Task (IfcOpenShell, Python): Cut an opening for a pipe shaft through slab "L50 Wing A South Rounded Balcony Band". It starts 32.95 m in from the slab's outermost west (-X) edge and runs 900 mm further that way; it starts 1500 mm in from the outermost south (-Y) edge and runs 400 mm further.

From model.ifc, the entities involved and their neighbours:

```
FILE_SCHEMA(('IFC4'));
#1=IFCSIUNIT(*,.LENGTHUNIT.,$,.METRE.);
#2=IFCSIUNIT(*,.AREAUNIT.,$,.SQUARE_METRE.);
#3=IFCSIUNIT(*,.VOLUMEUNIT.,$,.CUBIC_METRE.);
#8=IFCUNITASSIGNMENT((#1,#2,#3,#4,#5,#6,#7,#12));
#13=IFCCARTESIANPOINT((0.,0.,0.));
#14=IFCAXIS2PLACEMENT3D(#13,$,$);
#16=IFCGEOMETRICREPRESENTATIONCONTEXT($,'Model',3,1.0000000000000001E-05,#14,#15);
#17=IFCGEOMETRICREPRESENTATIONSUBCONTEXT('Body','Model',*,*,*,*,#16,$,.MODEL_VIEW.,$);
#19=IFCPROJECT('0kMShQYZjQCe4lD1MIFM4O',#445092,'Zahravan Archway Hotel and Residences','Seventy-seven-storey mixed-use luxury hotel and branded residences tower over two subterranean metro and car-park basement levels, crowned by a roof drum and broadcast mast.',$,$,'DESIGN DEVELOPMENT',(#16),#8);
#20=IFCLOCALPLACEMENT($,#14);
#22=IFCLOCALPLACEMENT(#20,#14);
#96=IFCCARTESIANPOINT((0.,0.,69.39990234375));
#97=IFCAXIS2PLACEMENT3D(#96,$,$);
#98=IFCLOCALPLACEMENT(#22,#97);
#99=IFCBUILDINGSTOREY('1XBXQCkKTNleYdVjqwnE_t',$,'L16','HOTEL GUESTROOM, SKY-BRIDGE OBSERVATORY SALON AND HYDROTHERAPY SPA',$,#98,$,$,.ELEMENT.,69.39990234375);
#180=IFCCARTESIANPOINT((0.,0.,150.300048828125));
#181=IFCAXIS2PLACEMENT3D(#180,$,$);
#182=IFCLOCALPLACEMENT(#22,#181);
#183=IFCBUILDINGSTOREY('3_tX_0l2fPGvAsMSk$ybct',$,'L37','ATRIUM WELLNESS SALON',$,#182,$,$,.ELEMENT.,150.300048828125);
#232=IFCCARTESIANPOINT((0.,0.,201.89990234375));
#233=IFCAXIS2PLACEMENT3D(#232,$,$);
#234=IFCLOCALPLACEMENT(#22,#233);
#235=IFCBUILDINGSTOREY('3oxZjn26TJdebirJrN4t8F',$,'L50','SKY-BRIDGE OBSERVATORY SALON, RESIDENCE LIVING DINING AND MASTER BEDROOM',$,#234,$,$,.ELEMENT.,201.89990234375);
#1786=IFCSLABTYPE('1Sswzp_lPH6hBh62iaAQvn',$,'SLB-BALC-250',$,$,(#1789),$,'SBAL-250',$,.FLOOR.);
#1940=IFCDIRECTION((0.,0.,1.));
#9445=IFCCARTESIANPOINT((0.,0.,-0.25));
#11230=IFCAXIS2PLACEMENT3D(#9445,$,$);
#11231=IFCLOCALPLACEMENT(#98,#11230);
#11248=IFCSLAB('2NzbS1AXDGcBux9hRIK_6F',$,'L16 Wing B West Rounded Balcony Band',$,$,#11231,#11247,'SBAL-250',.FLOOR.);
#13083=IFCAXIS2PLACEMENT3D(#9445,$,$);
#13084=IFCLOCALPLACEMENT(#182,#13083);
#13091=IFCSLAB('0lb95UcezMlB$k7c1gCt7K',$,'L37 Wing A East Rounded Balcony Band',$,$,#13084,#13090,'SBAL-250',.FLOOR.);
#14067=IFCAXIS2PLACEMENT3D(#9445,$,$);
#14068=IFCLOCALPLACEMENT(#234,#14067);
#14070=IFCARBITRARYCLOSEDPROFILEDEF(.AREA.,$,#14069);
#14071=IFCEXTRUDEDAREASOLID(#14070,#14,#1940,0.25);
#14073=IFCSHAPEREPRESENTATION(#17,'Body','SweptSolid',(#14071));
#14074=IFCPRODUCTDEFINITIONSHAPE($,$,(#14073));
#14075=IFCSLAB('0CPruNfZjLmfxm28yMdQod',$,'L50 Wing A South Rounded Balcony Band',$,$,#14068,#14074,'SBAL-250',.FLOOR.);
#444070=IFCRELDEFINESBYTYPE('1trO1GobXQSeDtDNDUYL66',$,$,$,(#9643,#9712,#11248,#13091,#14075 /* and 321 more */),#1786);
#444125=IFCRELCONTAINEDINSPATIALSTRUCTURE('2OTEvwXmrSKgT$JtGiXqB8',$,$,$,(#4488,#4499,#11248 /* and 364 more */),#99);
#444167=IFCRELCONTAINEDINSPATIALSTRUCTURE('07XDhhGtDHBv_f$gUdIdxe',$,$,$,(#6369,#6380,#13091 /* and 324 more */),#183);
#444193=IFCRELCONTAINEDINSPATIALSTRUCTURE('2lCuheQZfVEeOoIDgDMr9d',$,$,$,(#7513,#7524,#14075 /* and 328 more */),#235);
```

```python
import numpy as np
import ifcopenshell
import ifcopenshell.api.feature
import ifcopenshell.api.geometry
import ifcopenshell.api.root
import ifcopenshell.geom
import ifcopenshell.util.placement
import ifcopenshell.util.representation
import ifcopenshell.util.shape
import ifcopenshell.util.unit

model = ifcopenshell.open("model.ifc")
unit_scale = ifcopenshell.util.unit.calculate_unit_scale(model)
settings = ifcopenshell.geom.settings()


def volume(element):
    """Net volume in cubic metres, openings subtracted."""
    shape = ifcopenshell.geom.create_shape(settings, element)
    return ifcopenshell.util.shape.get_volume(shape.geometry)


slab = model.by_guid("0CPruNfZjLmfxm28yMdQod")
before = volume(slab)

# Extent in the slab's own axes, in metres. The edges named are its -X and -Y sides.
slab_shape = ifcopenshell.geom.create_shape(settings, slab)
vertices = ifcopenshell.util.shape.get_vertices(slab_shape.geometry)
x_min, y_min, bottom = vertices.min(axis=0)
top = vertices[:, 2].max()

opening = ifcopenshell.api.root.create_entity(model, ifc_class="IfcOpeningElement", name="Pipe shaft opening", predefined_type="OPENING")
context = ifcopenshell.util.representation.get_context(model, "Model", "Body", "MODEL_VIEW")
width, depth = 0.9, 0.4
outline = [(0.0, 0.0), (width, 0.0), (width, depth), (0.0, depth), (0.0, 0.0)]
# Overshoot both faces by 50 mm so the cut is clean.
shape = ifcopenshell.api.geometry.add_slab_representation(
    model, context=context, depth=top - bottom + 0.1, polyline=outline
)
ifcopenshell.api.geometry.assign_representation(model, product=opening, representation=shape)

matrix = ifcopenshell.util.placement.get_local_placement(slab.ObjectPlacement)
matrix[:, 3] = matrix @ np.append(np.array([x_min + 32.95, y_min + 1.5, bottom - 0.05]) / unit_scale, 1.0)
ifcopenshell.api.geometry.edit_object_placement(model, product=opening, matrix=matrix, is_si=False)
ifcopenshell.api.feature.add_feature(model, feature=opening, element=slab)

after = volume(slab)

print(f"slab volume {before:.3f} -> {after:.3f} m3")

model.write("model_edited.ifc")
```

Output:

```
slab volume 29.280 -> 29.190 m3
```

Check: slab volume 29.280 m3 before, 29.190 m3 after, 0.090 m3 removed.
